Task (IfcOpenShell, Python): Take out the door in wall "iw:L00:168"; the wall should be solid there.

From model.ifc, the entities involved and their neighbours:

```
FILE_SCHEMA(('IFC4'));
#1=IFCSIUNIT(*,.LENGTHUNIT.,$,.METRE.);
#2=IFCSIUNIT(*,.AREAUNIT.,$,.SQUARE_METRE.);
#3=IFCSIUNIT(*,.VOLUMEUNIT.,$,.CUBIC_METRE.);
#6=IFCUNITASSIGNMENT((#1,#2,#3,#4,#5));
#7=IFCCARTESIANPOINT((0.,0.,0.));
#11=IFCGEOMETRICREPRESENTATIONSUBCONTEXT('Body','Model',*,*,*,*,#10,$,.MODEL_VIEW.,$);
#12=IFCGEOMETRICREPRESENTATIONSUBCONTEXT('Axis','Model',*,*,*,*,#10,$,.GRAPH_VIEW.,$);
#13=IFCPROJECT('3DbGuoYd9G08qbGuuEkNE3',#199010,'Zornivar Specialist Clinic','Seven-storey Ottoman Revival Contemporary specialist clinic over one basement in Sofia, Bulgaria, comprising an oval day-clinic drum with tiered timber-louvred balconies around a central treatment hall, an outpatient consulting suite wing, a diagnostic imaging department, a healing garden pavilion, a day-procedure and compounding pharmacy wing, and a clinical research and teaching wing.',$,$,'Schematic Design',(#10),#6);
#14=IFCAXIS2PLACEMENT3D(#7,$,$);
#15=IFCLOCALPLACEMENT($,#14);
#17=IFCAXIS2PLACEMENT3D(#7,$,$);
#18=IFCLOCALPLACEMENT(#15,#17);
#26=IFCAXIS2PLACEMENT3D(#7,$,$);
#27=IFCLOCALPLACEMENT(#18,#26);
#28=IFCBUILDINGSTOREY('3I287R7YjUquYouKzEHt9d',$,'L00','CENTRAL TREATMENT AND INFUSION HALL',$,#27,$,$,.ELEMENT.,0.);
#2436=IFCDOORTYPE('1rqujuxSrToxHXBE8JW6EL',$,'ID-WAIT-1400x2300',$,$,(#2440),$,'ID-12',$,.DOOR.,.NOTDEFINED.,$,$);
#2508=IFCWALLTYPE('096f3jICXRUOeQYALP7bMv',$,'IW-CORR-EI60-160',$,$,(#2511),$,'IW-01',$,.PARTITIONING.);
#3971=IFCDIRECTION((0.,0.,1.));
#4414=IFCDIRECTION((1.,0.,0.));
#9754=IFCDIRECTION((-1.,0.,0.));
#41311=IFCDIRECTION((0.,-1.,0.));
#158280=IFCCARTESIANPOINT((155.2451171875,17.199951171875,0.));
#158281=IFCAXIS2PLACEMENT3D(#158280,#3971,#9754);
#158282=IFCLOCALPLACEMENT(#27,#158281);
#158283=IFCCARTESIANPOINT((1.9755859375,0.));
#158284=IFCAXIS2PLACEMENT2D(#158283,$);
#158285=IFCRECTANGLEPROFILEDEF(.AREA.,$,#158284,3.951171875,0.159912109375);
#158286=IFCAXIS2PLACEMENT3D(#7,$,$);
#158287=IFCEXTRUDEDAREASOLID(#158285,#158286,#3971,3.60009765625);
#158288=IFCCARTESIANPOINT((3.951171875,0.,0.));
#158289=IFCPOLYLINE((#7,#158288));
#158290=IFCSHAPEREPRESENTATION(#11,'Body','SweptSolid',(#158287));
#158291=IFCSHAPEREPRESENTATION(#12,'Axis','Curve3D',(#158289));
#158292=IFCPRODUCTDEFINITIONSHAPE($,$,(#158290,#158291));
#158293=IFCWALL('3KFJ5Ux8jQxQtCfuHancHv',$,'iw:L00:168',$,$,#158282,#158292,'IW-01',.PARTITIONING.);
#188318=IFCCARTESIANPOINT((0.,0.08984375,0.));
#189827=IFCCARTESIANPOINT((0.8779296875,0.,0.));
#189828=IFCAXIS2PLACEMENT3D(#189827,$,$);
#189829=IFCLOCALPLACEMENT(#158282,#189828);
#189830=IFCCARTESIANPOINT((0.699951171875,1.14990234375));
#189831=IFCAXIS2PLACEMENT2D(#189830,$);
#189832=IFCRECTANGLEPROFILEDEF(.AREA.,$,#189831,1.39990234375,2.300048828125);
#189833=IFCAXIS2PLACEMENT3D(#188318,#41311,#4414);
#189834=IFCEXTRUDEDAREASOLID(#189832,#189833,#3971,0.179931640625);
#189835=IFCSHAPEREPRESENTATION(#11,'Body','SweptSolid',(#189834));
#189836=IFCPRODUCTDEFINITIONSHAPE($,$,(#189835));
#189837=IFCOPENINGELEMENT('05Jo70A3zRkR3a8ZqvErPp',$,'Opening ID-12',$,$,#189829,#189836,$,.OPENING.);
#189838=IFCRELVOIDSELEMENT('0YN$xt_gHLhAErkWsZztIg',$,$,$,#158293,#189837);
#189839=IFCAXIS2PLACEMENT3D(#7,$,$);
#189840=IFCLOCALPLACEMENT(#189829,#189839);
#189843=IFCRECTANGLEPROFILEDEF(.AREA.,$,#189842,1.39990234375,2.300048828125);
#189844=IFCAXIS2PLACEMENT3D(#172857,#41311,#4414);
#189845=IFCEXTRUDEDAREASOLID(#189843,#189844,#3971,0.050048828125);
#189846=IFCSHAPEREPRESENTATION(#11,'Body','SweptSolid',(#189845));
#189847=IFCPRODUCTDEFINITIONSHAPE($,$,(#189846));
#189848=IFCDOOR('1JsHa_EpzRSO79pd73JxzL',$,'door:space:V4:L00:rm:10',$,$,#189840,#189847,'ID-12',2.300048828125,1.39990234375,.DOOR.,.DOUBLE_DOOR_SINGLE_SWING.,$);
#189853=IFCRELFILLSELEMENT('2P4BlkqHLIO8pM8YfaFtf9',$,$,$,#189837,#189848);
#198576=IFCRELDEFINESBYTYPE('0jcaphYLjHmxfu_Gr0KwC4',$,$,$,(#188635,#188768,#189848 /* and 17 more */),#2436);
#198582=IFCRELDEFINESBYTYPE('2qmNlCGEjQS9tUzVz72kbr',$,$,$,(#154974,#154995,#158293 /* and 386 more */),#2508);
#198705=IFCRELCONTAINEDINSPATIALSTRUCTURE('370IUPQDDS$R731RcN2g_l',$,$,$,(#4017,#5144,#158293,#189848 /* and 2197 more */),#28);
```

```python
import ifcopenshell
import ifcopenshell.api.feature
import ifcopenshell.api.root
import ifcopenshell.geom
import ifcopenshell.util.shape

model = ifcopenshell.open("model.ifc")
settings = ifcopenshell.geom.settings()


def volume(element):
    """Net volume in cubic metres, openings subtracted."""
    shape = ifcopenshell.geom.create_shape(settings, element)
    return ifcopenshell.util.shape.get_volume(shape.geometry)


door = model.by_guid("1JsHa_EpzRSO79pd73JxzL")
opening = door.FillsVoids[0].RelatingOpeningElement
wall = opening.VoidsElements[0].RelatingBuildingElement
before = volume(wall)

ifcopenshell.api.root.remove_product(model, product=door)
ifcopenshell.api.feature.remove_feature(model, feature=opening)

after = volume(wall)

print(f"wall volume {before:.3f} -> {after:.3f} m3")

model.write("model_v2.ifc")
```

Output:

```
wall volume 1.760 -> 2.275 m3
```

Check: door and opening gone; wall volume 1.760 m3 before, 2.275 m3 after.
